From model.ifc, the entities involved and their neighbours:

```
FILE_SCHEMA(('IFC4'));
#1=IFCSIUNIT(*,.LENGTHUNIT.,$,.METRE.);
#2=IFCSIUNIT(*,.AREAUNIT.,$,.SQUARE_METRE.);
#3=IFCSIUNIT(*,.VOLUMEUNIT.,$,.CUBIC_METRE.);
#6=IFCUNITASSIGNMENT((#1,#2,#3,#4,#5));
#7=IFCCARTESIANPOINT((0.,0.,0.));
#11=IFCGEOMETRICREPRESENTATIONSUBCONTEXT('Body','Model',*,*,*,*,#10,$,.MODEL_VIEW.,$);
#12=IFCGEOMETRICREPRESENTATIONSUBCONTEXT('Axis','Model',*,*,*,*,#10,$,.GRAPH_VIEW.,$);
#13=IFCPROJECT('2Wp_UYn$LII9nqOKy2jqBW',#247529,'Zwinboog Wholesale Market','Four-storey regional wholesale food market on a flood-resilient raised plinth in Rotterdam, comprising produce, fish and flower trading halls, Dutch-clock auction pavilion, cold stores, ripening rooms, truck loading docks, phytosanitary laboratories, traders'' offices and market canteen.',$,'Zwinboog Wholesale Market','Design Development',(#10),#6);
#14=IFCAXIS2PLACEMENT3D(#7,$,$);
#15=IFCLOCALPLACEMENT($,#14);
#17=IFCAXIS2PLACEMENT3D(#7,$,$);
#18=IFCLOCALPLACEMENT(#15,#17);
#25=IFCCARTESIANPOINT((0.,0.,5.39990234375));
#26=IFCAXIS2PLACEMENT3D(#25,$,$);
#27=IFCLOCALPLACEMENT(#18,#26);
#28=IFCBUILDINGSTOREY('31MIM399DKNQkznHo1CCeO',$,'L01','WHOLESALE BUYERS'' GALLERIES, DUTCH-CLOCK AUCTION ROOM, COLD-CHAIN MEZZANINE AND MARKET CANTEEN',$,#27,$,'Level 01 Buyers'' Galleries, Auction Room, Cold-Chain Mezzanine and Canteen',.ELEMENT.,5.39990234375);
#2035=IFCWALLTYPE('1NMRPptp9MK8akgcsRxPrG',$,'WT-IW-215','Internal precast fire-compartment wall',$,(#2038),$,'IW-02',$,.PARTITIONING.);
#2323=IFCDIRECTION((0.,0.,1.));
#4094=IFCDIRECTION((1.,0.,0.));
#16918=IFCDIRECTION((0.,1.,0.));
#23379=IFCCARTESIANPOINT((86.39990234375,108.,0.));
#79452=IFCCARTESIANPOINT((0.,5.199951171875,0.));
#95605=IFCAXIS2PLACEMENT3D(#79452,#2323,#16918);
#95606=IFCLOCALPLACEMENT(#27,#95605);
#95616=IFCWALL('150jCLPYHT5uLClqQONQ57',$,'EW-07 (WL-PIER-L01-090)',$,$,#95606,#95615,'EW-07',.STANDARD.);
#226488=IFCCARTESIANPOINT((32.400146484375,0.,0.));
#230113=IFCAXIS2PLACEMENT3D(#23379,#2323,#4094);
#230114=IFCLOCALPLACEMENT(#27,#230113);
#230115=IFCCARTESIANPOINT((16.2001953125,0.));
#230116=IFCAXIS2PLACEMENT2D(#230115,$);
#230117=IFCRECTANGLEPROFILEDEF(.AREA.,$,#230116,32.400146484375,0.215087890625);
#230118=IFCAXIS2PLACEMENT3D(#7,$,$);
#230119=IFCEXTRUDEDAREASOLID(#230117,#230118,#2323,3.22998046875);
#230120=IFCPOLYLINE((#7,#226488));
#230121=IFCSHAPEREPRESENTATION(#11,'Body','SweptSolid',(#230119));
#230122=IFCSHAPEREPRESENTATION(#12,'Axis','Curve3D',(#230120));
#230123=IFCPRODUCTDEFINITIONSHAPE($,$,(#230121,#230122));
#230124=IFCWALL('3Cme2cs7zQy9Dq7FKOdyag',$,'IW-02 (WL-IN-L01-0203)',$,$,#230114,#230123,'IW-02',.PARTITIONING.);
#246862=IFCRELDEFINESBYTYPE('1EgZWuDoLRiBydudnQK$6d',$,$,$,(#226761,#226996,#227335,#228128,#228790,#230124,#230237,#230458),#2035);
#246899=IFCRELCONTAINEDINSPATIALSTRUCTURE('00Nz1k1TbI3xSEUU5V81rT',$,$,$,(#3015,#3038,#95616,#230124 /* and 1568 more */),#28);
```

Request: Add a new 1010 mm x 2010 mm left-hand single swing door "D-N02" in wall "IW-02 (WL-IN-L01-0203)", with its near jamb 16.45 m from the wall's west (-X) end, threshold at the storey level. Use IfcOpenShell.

```python
import numpy as np
import ifcopenshell
import ifcopenshell.api.feature
import ifcopenshell.api.geometry
import ifcopenshell.api.root
import ifcopenshell.api.spatial
import ifcopenshell.geom
import ifcopenshell.util.element
import ifcopenshell.util.placement
import ifcopenshell.util.representation
import ifcopenshell.util.shape
import ifcopenshell.util.unit

model = ifcopenshell.open("model.ifc")
unit_scale = ifcopenshell.util.unit.calculate_unit_scale(model)
settings = ifcopenshell.geom.settings()


def volume(element):
    """Net volume in cubic metres, openings subtracted."""
    shape = ifcopenshell.geom.create_shape(settings, element)
    return ifcopenshell.util.shape.get_volume(shape.geometry)


wall = model.by_guid("3Cme2cs7zQy9Dq7FKOdyag")
storey = ifcopenshell.util.element.get_container(wall, ifc_class="IfcBuildingStorey")
context = ifcopenshell.util.representation.get_context(model, "Model", "Body", "MODEL_VIEW")
before = volume(wall)

width, height, from_end, sill = 1.01, 2.01, 16.45, 0.0  # metres

# The wall runs along its own X axis, and the end named is its -X end.
wall_shape = ifcopenshell.geom.create_shape(settings, wall)
x, y, z = ifcopenshell.util.shape.get_vertices(wall_shape.geometry).T
start = x.min() + from_end
face, thickness = float(y.min()), float(y.max() - y.min())
wall_matrix = ifcopenshell.util.placement.get_local_placement(wall.ObjectPlacement)
level = ifcopenshell.util.placement.get_local_placement(storey.ObjectPlacement)[2, 3]


def in_wall(x, y):
    """Placement at x, y metres in the wall's axes, at sill height."""
    matrix = wall_matrix.copy()
    matrix[:, 3] = wall_matrix @ np.array([x / unit_scale, y / unit_scale, 0.0, 1.0])
    matrix[2, 3] = level + sill / unit_scale
    return matrix


# Opening: a box that overshoots both wall faces by 50 mm.
opening = ifcopenshell.api.root.create_entity(model, ifc_class="IfcOpeningElement", predefined_type="OPENING")
box = ifcopenshell.api.geometry.add_wall_representation(
    model, context=context, length=width, height=height, thickness=thickness + 0.1
)
ifcopenshell.api.geometry.assign_representation(model, product=opening, representation=box)
ifcopenshell.api.geometry.edit_object_placement(model, product=opening, matrix=in_wall(start, face - 0.05), is_si=False)
ifcopenshell.api.feature.add_feature(model, feature=opening, element=wall)

door = ifcopenshell.api.root.create_entity(model, ifc_class="IfcDoor", name="D-N02", predefined_type="DOOR")
door.OverallWidth, door.OverallHeight = width / unit_scale, height / unit_scale
door.OperationType = "SINGLE_SWING_LEFT"
body = ifcopenshell.api.geometry.add_door_representation(
    model,
    context=context,
    overall_width=door.OverallWidth,
    overall_height=door.OverallHeight,
    operation_type="SINGLE_SWING_LEFT",
    lining_properties={"LiningDepth": thickness / unit_scale, "ThresholdDepth": thickness / unit_scale},
)
ifcopenshell.api.geometry.assign_representation(model, product=door, representation=body)
ifcopenshell.api.spatial.assign_container(model, products=[door], relating_structure=storey)
ifcopenshell.api.feature.add_filling(model, opening=opening, element=door)

# The lining spans the wall, so the door starts at the wall face.
ifcopenshell.api.geometry.edit_object_placement(model, product=door, matrix=in_wall(start, face), is_si=False)

after = volume(wall)

print(f"wall volume {before:.3f} -> {after:.3f} m3")

model.write("model_edited.ifc")
```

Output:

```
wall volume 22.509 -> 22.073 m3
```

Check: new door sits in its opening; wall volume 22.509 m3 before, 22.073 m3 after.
